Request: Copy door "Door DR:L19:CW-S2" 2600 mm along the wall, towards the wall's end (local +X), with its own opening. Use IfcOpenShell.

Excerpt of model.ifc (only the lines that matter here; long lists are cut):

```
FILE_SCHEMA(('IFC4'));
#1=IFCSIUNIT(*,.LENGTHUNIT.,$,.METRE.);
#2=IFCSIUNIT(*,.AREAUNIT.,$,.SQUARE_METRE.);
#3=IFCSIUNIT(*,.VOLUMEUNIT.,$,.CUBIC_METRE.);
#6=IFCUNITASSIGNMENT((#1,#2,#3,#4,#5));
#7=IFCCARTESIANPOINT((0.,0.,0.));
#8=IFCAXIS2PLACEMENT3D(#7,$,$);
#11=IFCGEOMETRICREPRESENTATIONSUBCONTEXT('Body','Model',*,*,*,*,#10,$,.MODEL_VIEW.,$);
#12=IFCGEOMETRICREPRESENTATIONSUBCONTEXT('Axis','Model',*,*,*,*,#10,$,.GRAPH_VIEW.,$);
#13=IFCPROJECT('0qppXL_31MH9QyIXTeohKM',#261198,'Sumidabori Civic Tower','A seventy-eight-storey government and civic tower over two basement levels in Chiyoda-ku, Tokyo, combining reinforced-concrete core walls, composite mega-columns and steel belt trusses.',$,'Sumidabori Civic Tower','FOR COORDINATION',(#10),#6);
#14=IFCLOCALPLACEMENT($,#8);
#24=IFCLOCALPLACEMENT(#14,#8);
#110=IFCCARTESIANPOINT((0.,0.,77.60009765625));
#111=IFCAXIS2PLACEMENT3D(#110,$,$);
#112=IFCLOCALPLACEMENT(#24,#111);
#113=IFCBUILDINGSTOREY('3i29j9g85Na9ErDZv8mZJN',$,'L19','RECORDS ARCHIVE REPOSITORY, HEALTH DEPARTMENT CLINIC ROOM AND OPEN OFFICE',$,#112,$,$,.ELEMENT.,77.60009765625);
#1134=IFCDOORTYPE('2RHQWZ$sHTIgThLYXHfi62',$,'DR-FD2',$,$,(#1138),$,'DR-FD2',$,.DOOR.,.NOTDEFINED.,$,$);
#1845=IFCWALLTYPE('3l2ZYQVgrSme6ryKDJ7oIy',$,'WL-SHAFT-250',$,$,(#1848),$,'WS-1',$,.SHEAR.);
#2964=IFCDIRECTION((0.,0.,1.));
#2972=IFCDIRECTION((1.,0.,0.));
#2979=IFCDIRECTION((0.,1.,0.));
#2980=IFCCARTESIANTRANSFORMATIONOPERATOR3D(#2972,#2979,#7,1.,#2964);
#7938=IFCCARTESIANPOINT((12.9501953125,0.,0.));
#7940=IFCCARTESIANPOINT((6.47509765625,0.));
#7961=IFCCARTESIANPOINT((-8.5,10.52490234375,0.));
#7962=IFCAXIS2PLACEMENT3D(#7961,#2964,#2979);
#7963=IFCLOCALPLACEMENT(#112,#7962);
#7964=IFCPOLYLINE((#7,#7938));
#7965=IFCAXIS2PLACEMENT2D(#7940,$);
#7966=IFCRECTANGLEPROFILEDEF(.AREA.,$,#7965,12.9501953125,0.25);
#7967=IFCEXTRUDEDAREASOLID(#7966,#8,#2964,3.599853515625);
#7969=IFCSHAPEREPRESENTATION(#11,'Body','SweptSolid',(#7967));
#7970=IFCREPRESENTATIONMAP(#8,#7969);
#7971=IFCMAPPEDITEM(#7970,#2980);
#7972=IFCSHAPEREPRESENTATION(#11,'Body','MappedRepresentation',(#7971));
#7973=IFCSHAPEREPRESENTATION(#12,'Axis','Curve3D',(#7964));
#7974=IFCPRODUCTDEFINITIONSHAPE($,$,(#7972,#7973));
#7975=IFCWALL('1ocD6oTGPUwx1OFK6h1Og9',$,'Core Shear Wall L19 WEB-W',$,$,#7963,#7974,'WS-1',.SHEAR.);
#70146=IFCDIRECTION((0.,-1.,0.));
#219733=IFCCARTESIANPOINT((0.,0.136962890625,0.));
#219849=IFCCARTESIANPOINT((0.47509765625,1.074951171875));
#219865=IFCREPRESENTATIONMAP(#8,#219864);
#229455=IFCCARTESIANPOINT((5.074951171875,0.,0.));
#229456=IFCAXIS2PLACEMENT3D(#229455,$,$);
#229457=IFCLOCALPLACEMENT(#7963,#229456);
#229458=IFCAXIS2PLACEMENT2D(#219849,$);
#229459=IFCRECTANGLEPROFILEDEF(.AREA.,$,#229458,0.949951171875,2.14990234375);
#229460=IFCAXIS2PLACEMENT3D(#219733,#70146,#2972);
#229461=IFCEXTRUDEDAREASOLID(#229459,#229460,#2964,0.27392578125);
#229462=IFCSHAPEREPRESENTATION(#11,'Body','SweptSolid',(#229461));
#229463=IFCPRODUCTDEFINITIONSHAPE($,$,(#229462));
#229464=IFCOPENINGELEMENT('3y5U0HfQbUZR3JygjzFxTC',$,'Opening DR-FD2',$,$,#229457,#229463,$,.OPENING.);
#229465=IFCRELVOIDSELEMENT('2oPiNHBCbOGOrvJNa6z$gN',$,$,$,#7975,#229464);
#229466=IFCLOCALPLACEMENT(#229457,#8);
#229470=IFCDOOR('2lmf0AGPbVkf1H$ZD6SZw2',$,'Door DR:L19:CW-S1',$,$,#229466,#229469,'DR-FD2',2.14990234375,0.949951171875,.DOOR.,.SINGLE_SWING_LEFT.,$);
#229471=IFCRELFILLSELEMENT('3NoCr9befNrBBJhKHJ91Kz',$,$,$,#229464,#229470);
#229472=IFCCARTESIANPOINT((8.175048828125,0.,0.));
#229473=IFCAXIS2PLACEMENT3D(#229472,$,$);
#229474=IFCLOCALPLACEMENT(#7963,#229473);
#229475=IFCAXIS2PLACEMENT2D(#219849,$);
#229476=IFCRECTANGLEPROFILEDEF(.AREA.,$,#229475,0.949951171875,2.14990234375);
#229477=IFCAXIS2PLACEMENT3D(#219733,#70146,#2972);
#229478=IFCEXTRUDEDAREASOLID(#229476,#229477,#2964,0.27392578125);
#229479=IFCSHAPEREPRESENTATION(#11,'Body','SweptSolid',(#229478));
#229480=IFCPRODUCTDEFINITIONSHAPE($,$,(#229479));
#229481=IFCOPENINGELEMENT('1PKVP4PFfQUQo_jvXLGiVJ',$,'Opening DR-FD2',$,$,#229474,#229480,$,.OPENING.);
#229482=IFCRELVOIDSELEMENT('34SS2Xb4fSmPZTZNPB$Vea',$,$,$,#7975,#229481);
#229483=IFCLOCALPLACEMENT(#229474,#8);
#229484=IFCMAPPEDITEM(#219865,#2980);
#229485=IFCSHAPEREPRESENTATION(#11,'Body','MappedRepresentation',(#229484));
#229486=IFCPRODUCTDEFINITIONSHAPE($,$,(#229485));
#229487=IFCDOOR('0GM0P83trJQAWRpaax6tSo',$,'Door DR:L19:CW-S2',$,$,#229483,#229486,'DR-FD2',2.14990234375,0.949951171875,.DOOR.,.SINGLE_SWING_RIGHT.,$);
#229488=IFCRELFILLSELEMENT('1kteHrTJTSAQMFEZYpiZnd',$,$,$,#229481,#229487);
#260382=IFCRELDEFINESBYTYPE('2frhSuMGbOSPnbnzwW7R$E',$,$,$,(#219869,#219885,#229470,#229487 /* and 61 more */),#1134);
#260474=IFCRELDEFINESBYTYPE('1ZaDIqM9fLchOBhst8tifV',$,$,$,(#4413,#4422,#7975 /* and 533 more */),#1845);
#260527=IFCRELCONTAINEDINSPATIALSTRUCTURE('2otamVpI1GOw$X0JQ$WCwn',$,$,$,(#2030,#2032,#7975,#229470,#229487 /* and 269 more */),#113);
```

```python
import ifcopenshell
import ifcopenshell.api.feature
import ifcopenshell.api.geometry
import ifcopenshell.api.root
import ifcopenshell.geom
import ifcopenshell.util.element
import ifcopenshell.util.placement
import ifcopenshell.util.shape

model = ifcopenshell.open("model.ifc")
settings = ifcopenshell.geom.settings()


def volume(element):
    """Net volume in cubic metres, openings subtracted."""
    shape = ifcopenshell.geom.create_shape(settings, element)
    return ifcopenshell.util.shape.get_volume(shape.geometry)


door = model.by_guid("0GM0P83trJQAWRpaax6tSo")
opening = door.FillsVoids[0].RelatingOpeningElement
wall = opening.VoidsElements[0].RelatingBuildingElement
before = volume(wall)
shift = ifcopenshell.util.placement.get_local_placement(wall.ObjectPlacement)[:3, 0] * 2.6

# copy_class copies the void relationship, type, container and properties, but no geometry.
new_opening = ifcopenshell.api.root.copy_class(model, product=opening)
new_opening.Representation = ifcopenshell.util.element.copy_deep(
    model, opening.Representation, exclude=["IfcGeometricRepresentationContext", "IfcRepresentationMap"]
)
new_door = ifcopenshell.api.root.copy_class(model, product=door)
new_door.Representation = ifcopenshell.util.element.copy_deep(
    model, door.Representation, exclude=["IfcGeometricRepresentationContext", "IfcRepresentationMap"]
)
new_door.Tag = None
ifcopenshell.api.feature.add_filling(model, opening=new_opening, element=new_door)

for old, new in ((opening, new_opening), (door, new_door)):
    matrix = ifcopenshell.util.placement.get_local_placement(old.ObjectPlacement)
    matrix[:3, 3] += shift
    ifcopenshell.api.geometry.edit_object_placement(model, product=new, matrix=matrix, is_si=False)

after = volume(wall)

print(f"wall volume {before:.3f} -> {after:.3f} m3")

model.write("model_edited.ifc")
```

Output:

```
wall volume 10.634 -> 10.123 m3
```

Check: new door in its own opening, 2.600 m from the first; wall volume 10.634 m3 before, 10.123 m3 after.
